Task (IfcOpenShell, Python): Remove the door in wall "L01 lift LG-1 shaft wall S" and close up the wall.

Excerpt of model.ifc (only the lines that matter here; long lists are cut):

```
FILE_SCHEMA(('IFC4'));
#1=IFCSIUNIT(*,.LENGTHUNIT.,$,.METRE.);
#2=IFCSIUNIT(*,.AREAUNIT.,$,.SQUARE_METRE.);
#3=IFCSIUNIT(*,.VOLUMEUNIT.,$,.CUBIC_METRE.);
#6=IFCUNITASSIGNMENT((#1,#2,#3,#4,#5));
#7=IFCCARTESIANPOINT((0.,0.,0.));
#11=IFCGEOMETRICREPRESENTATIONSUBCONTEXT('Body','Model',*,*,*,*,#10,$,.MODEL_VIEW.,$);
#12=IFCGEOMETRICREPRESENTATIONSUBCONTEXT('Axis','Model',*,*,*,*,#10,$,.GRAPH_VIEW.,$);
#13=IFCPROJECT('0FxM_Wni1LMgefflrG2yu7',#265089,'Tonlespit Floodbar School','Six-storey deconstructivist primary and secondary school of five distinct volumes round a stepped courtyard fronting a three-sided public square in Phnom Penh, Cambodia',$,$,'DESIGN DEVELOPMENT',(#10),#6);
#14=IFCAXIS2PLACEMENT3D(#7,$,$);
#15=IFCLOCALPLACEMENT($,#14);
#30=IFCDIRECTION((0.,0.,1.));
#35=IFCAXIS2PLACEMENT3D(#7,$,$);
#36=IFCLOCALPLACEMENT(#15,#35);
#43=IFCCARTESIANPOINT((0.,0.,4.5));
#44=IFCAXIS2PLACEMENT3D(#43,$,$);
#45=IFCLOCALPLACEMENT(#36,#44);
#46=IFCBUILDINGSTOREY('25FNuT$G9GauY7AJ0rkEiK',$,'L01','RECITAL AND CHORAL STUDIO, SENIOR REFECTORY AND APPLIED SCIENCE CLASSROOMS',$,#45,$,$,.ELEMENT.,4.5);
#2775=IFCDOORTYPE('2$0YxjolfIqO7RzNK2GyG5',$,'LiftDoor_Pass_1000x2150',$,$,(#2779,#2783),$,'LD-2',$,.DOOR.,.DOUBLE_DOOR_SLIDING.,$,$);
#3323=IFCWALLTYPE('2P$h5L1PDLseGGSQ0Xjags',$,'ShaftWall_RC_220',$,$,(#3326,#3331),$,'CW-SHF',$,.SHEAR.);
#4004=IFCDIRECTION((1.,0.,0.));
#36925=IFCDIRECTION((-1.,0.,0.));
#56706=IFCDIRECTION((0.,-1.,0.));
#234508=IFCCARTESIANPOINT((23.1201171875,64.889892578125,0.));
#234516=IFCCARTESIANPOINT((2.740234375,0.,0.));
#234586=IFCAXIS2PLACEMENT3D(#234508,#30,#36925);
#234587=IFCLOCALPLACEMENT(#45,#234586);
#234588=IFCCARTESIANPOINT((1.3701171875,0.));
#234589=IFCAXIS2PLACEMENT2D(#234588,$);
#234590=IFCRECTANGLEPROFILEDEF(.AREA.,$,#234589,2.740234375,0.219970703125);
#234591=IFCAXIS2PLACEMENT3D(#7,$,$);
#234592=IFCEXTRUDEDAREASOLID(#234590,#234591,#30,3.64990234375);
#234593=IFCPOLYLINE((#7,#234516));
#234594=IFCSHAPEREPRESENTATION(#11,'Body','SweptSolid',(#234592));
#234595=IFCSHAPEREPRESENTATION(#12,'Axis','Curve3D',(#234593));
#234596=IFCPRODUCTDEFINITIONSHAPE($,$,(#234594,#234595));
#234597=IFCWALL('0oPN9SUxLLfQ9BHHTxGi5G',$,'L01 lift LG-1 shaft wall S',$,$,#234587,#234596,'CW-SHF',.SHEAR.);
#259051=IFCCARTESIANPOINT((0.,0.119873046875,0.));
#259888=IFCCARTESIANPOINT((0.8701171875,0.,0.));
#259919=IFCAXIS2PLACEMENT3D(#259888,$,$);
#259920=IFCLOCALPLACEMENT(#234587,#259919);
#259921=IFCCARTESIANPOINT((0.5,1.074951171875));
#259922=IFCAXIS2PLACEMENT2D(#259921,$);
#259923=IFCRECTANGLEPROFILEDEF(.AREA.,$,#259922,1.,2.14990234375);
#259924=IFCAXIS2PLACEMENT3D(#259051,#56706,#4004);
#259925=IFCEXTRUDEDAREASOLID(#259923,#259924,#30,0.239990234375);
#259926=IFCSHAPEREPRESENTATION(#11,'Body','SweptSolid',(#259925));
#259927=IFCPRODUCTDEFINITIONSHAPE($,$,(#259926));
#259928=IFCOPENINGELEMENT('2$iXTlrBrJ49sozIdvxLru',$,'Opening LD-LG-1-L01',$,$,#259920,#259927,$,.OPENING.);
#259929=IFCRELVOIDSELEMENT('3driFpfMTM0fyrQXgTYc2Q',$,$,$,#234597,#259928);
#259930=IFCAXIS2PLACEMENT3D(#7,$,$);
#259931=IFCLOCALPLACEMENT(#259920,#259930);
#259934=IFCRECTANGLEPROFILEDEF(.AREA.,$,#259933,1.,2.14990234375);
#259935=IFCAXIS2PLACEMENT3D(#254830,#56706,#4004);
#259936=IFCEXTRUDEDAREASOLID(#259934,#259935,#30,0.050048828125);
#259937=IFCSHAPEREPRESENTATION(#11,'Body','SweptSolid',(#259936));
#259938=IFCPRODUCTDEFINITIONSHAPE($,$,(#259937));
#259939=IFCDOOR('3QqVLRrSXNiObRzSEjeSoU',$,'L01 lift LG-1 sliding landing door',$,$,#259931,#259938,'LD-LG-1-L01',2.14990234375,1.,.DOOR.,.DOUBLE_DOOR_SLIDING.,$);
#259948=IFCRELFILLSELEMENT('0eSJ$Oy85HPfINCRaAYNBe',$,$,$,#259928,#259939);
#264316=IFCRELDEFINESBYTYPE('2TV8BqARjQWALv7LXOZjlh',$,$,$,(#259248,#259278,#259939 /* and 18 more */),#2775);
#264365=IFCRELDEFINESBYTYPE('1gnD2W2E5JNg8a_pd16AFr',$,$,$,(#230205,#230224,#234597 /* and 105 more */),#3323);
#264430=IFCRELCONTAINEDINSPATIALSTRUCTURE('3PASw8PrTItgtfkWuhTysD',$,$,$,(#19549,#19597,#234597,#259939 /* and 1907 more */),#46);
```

```python
import ifcopenshell
import ifcopenshell.api.feature
import ifcopenshell.api.root
import ifcopenshell.geom
import ifcopenshell.util.shape

model = ifcopenshell.open("model.ifc")
settings = ifcopenshell.geom.settings()


def volume(element):
    """Net volume in cubic metres, openings subtracted."""
    shape = ifcopenshell.geom.create_shape(settings, element)
    return ifcopenshell.util.shape.get_volume(shape.geometry)


door = model.by_guid("3QqVLRrSXNiObRzSEjeSoU")
opening = door.FillsVoids[0].RelatingOpeningElement
wall = opening.VoidsElements[0].RelatingBuildingElement
before = volume(wall)

ifcopenshell.api.root.remove_product(model, product=door)
ifcopenshell.api.feature.remove_feature(model, feature=opening)

after = volume(wall)

print(f"wall volume {before:.3f} -> {after:.3f} m3")

model.write("model-out.ifc")
```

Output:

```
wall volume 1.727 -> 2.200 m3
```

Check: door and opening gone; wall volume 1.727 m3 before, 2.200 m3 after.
